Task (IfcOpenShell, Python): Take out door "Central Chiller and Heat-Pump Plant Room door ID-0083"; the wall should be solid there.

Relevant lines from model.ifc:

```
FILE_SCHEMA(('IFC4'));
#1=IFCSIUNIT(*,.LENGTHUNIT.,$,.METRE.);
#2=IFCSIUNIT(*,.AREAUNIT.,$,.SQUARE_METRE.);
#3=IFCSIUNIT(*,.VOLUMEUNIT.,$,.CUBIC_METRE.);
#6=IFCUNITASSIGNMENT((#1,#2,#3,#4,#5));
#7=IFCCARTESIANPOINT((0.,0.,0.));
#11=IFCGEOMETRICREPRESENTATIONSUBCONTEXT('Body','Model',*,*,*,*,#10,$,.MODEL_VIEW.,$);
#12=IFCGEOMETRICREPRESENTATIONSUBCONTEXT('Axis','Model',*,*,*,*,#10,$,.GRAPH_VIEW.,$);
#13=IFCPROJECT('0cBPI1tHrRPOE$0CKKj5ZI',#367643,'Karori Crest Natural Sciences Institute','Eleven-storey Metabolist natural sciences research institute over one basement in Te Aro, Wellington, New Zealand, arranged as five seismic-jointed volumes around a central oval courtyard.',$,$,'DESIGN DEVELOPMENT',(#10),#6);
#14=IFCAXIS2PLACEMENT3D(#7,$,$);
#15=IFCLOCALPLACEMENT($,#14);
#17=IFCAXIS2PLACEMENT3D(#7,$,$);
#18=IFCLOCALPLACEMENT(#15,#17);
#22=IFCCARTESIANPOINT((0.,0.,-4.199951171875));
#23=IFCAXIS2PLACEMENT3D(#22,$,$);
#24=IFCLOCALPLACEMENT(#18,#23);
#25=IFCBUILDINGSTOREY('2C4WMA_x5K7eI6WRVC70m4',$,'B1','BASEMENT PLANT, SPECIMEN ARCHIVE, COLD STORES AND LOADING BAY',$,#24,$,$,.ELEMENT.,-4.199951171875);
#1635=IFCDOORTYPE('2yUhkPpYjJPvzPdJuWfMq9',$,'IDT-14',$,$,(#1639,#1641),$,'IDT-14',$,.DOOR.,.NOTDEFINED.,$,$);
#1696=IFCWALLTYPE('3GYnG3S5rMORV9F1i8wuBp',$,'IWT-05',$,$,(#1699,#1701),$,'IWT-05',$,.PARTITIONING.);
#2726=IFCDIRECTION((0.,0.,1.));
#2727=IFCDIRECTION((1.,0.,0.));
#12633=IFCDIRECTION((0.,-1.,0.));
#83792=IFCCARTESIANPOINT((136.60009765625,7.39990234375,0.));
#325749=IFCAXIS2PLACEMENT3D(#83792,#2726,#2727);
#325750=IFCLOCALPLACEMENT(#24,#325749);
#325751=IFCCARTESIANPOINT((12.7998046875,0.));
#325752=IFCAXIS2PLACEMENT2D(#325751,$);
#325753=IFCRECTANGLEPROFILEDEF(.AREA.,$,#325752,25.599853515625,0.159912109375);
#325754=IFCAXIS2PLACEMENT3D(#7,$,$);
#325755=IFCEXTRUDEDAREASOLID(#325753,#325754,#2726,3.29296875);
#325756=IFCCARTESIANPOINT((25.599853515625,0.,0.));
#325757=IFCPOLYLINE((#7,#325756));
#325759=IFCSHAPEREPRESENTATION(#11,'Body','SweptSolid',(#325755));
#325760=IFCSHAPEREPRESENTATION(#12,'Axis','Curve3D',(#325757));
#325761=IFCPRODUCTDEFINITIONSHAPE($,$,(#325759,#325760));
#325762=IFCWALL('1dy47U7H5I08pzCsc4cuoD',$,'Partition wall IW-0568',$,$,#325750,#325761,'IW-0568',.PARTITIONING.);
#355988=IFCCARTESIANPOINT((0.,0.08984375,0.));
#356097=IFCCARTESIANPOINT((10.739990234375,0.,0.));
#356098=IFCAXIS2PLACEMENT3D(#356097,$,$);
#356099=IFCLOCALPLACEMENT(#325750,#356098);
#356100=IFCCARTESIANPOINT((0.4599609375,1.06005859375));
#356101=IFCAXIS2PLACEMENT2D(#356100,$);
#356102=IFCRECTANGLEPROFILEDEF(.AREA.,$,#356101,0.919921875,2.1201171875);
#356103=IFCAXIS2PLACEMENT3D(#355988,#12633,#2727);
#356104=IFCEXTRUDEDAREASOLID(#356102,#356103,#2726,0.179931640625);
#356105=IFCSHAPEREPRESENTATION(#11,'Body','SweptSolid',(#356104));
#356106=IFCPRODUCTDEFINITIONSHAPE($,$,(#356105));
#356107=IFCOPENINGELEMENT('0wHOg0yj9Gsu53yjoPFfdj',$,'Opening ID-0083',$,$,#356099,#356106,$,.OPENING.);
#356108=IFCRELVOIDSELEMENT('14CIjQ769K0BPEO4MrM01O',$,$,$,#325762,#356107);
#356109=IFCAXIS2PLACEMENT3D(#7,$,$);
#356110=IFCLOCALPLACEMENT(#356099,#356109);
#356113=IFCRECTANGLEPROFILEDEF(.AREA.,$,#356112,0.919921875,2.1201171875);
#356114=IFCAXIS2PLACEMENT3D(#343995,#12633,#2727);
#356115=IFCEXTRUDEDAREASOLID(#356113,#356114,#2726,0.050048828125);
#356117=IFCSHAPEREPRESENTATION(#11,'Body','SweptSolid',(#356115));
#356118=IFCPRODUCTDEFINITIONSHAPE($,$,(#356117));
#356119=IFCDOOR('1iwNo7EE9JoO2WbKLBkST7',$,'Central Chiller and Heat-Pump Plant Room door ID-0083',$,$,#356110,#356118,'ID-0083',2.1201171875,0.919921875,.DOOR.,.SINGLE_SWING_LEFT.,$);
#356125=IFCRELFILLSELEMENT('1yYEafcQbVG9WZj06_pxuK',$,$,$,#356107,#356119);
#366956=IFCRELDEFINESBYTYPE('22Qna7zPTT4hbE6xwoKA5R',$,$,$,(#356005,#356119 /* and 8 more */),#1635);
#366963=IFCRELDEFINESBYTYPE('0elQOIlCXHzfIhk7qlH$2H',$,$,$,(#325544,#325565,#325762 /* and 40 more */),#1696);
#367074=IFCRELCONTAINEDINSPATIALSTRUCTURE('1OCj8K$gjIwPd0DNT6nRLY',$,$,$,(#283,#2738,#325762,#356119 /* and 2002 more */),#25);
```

```python
import ifcopenshell
import ifcopenshell.api.feature
import ifcopenshell.api.root
import ifcopenshell.geom
import ifcopenshell.util.shape

model = ifcopenshell.open("model.ifc")
settings = ifcopenshell.geom.settings()


def volume(element):
    """Net volume in cubic metres, openings subtracted."""
    shape = ifcopenshell.geom.create_shape(settings, element)
    return ifcopenshell.util.shape.get_volume(shape.geometry)


door = model.by_guid("1iwNo7EE9JoO2WbKLBkST7")
opening = door.FillsVoids[0].RelatingOpeningElement
wall = opening.VoidsElements[0].RelatingBuildingElement
before = volume(wall)

ifcopenshell.api.root.remove_product(model, product=door)
ifcopenshell.api.feature.remove_feature(model, feature=opening)

after = volume(wall)

print(f"wall volume {before:.3f} -> {after:.3f} m3")

model.write("model_v2.ifc")
```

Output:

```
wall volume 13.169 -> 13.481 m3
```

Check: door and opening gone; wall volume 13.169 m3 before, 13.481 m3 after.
